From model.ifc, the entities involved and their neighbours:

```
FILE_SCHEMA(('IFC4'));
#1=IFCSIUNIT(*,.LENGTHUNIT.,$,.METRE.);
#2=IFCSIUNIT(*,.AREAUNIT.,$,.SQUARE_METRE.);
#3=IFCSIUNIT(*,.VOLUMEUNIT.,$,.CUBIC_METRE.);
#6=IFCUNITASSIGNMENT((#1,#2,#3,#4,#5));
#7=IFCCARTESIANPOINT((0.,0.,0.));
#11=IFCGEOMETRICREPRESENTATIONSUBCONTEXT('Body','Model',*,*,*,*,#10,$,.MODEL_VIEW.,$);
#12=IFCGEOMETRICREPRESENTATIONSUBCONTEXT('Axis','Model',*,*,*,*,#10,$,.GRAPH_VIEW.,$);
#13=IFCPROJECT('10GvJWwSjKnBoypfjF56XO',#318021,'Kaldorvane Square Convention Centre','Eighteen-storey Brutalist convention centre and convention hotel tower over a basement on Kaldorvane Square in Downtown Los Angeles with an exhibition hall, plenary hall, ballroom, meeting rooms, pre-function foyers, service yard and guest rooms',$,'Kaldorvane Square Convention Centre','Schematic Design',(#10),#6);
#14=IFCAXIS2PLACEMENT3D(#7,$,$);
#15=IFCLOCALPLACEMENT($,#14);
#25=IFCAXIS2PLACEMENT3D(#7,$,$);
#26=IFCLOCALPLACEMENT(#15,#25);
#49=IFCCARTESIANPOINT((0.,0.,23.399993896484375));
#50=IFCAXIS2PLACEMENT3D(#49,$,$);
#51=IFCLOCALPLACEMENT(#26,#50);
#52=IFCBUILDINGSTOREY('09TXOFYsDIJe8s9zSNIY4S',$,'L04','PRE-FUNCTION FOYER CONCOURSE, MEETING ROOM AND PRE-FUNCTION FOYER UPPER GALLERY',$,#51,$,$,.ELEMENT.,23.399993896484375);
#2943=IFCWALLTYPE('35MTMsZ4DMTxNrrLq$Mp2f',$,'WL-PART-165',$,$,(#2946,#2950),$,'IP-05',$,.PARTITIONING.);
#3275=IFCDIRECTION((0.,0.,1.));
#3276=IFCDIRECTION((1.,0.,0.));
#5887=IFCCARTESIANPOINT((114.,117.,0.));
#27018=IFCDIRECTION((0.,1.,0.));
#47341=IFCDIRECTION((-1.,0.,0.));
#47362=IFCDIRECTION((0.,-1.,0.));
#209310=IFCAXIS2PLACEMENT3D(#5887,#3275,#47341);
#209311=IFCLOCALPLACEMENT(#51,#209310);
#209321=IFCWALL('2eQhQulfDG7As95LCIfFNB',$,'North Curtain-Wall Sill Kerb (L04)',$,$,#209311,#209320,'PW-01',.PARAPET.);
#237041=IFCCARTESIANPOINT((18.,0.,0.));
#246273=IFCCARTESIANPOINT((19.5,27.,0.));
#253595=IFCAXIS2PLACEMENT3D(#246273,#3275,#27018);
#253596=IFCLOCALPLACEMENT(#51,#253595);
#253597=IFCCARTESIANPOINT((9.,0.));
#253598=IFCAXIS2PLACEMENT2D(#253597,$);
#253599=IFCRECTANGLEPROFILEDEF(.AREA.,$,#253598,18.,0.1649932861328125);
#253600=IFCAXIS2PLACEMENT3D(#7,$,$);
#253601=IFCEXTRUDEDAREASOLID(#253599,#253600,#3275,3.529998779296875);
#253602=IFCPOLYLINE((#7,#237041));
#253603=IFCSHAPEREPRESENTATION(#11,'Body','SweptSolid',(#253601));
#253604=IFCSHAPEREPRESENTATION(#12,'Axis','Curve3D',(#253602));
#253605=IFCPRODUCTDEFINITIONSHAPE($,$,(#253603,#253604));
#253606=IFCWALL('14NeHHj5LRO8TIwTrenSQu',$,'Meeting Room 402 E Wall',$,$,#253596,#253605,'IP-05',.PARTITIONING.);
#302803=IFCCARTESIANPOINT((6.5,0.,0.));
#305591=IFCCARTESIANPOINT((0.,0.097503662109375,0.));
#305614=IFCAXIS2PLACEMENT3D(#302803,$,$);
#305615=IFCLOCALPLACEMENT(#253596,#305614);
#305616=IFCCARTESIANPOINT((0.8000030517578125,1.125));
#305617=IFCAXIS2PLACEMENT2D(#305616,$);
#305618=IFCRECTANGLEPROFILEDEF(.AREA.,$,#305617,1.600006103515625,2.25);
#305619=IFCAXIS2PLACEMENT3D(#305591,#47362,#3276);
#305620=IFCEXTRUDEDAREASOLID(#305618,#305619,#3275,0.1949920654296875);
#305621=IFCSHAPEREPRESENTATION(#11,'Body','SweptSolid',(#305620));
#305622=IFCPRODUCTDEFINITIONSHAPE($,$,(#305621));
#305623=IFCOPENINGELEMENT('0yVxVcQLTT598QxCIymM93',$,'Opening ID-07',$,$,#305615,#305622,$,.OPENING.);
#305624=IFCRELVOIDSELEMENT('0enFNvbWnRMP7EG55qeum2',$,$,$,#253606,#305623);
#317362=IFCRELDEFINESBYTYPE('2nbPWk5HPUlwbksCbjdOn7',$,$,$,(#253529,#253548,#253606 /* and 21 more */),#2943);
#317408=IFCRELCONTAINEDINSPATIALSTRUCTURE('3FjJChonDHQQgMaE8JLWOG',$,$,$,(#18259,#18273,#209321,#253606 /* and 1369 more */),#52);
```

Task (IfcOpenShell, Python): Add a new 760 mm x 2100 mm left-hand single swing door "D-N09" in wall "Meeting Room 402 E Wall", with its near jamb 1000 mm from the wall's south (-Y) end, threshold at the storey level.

```python
import numpy as np
import ifcopenshell
import ifcopenshell.api.feature
import ifcopenshell.api.geometry
import ifcopenshell.api.root
import ifcopenshell.api.spatial
import ifcopenshell.geom
import ifcopenshell.util.element
import ifcopenshell.util.placement
import ifcopenshell.util.representation
import ifcopenshell.util.shape
import ifcopenshell.util.unit

model = ifcopenshell.open("model.ifc")
unit_scale = ifcopenshell.util.unit.calculate_unit_scale(model)
settings = ifcopenshell.geom.settings()


def volume(element):
    """Net volume in cubic metres, openings subtracted."""
    shape = ifcopenshell.geom.create_shape(settings, element)
    return ifcopenshell.util.shape.get_volume(shape.geometry)


wall = model.by_id(253606)
storey = ifcopenshell.util.element.get_container(wall, ifc_class="IfcBuildingStorey")
context = ifcopenshell.util.representation.get_context(model, "Model", "Body", "MODEL_VIEW")
before = volume(wall)

width, height, from_end, sill = 0.76, 2.1, 1, 0.0  # metres

# The wall runs along its own X axis, and the end named is its -X end.
wall_shape = ifcopenshell.geom.create_shape(settings, wall)
x, y, z = ifcopenshell.util.shape.get_vertices(wall_shape.geometry).T
start = x.min() + from_end
face, thickness = float(y.min()), float(y.max() - y.min())
wall_matrix = ifcopenshell.util.placement.get_local_placement(wall.ObjectPlacement)
level = ifcopenshell.util.placement.get_local_placement(storey.ObjectPlacement)[2, 3]


def in_wall(x, y):
    """Placement at x, y metres in the wall's axes, at sill height."""
    matrix = wall_matrix.copy()
    matrix[:, 3] = wall_matrix @ np.array([x / unit_scale, y / unit_scale, 0.0, 1.0])
    matrix[2, 3] = level + sill / unit_scale
    return matrix


# Opening: a box that overshoots both wall faces by 50 mm.
opening = ifcopenshell.api.root.create_entity(model, ifc_class="IfcOpeningElement", predefined_type="OPENING")
box = ifcopenshell.api.geometry.add_wall_representation(
    model, context=context, length=width, height=height, thickness=thickness + 0.1
)
ifcopenshell.api.geometry.assign_representation(model, product=opening, representation=box)
ifcopenshell.api.geometry.edit_object_placement(model, product=opening, matrix=in_wall(start, face - 0.05), is_si=False)
ifcopenshell.api.feature.add_feature(model, feature=opening, element=wall)

door = ifcopenshell.api.root.create_entity(model, ifc_class="IfcDoor", name="D-N09", predefined_type="DOOR")
door.OverallWidth, door.OverallHeight = width / unit_scale, height / unit_scale
door.OperationType = "SINGLE_SWING_LEFT"
body = ifcopenshell.api.geometry.add_door_representation(
    model,
    context=context,
    overall_width=door.OverallWidth,
    overall_height=door.OverallHeight,
    operation_type="SINGLE_SWING_LEFT",
    lining_properties={"LiningDepth": thickness / unit_scale, "ThresholdDepth": thickness / unit_scale},
)
ifcopenshell.api.geometry.assign_representation(model, product=door, representation=body)
ifcopenshell.api.spatial.assign_container(model, products=[door], relating_structure=storey)
ifcopenshell.api.feature.add_filling(model, opening=opening, element=door)

# The lining spans the wall, so the door starts at the wall face.
ifcopenshell.api.geometry.edit_object_placement(model, product=door, matrix=in_wall(start, face), is_si=False)

after = volume(wall)

print(f"wall volume {before:.3f} -> {after:.3f} m3")

model.write("model_updated.ifc")
```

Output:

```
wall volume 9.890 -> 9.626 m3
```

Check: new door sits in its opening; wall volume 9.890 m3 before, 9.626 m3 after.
